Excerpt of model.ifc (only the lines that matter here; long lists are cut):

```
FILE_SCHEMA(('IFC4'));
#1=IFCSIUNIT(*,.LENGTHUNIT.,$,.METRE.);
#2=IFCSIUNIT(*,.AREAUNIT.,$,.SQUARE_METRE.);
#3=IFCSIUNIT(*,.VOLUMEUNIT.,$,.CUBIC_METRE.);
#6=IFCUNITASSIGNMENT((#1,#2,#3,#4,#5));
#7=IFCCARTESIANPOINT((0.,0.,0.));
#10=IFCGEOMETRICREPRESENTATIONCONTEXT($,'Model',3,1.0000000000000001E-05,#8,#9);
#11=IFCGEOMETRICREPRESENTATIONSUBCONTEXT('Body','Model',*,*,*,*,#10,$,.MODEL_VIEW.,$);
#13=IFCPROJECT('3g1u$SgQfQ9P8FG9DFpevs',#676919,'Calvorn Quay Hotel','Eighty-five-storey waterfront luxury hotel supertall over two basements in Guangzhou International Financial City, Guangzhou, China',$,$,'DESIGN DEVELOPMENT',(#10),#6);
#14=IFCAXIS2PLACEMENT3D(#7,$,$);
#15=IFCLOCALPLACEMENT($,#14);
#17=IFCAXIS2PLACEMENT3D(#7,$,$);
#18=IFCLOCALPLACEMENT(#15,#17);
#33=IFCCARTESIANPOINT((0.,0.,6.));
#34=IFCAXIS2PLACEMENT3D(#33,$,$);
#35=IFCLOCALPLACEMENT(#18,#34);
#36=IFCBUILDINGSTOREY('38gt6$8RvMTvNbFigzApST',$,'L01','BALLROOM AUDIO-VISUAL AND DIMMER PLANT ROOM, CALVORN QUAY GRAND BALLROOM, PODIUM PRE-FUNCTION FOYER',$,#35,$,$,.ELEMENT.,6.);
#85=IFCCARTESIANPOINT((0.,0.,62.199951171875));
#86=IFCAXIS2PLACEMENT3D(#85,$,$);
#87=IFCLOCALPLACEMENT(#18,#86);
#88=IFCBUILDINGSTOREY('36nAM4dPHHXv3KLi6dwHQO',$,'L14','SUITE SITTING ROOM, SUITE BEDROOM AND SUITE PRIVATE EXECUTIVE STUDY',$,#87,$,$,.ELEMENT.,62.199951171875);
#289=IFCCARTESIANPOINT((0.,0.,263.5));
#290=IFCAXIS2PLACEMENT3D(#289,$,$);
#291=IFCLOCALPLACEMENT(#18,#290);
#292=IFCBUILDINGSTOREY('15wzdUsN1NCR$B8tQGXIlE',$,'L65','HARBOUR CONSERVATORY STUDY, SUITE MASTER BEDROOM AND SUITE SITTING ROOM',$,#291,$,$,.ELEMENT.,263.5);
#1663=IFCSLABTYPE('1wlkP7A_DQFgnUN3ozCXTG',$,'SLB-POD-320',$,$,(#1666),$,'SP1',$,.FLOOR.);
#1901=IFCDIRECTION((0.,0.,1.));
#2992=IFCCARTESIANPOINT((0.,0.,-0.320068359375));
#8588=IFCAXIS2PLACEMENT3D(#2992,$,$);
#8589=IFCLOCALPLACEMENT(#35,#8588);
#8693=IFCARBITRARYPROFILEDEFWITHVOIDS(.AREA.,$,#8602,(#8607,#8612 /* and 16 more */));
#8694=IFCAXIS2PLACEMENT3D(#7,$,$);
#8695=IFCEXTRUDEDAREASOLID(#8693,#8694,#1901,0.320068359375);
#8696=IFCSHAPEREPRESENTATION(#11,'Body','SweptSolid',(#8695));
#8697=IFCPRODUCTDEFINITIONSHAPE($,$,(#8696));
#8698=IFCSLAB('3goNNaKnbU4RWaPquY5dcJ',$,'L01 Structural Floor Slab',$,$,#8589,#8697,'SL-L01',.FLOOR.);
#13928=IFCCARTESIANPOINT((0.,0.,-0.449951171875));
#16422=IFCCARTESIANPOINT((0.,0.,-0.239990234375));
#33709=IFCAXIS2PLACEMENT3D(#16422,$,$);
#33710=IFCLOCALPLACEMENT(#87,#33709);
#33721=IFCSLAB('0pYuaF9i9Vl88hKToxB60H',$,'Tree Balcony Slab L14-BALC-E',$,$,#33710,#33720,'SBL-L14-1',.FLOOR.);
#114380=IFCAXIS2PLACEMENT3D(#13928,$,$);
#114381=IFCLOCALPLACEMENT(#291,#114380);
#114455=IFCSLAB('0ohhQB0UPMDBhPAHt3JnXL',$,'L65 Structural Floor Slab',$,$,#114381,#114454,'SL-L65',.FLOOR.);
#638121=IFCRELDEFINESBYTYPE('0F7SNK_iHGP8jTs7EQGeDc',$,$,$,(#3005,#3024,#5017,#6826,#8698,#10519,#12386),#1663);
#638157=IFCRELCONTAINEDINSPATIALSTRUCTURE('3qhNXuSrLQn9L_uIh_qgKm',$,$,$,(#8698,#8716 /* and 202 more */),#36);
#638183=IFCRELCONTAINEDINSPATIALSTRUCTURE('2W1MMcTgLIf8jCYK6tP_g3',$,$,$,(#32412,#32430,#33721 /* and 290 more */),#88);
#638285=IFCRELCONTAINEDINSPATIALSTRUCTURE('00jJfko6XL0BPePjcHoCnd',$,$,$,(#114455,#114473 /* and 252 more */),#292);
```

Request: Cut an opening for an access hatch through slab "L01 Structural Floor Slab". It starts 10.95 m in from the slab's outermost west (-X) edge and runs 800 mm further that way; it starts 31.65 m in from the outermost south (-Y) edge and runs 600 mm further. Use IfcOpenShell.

```python
import numpy as np
import ifcopenshell
import ifcopenshell.api.feature
import ifcopenshell.api.geometry
import ifcopenshell.api.root
import ifcopenshell.geom
import ifcopenshell.util.placement
import ifcopenshell.util.representation
import ifcopenshell.util.shape
import ifcopenshell.util.unit

model = ifcopenshell.open("model.ifc")
unit_scale = ifcopenshell.util.unit.calculate_unit_scale(model)
settings = ifcopenshell.geom.settings()


def volume(element):
    """Net volume in cubic metres, openings subtracted."""
    shape = ifcopenshell.geom.create_shape(settings, element)
    return ifcopenshell.util.shape.get_volume(shape.geometry)


slab = model.by_guid("3goNNaKnbU4RWaPquY5dcJ")
before = volume(slab)

# Extent in the slab's own axes, in metres. The edges named are its -X and -Y sides.
slab_shape = ifcopenshell.geom.create_shape(settings, slab)
vertices = ifcopenshell.util.shape.get_vertices(slab_shape.geometry)
x_min, y_min, bottom = vertices.min(axis=0)
top = vertices[:, 2].max()

opening = ifcopenshell.api.root.create_entity(model, ifc_class="IfcOpeningElement", name="Access hatch opening", predefined_type="OPENING")
context = ifcopenshell.util.representation.get_context(model, "Model", "Body", "MODEL_VIEW")
width, depth = 0.8, 0.6
outline = [(0.0, 0.0), (width, 0.0), (width, depth), (0.0, depth), (0.0, 0.0)]
# Overshoot both faces by 50 mm so the cut is clean.
shape = ifcopenshell.api.geometry.add_slab_representation(
    model, context=context, depth=top - bottom + 0.1, polyline=outline
)
ifcopenshell.api.geometry.assign_representation(model, product=opening, representation=shape)

matrix = ifcopenshell.util.placement.get_local_placement(slab.ObjectPlacement)
matrix[:, 3] = matrix @ np.append(np.array([x_min + 10.95, y_min + 31.65, bottom - 0.05]) / unit_scale, 1.0)
ifcopenshell.api.geometry.edit_object_placement(model, product=opening, matrix=matrix, is_si=False)
ifcopenshell.api.feature.add_feature(model, feature=opening, element=slab)

after = volume(slab)

print(f"slab volume {before:.3f} -> {after:.3f} m3")

model.write("model-out.ifc")
```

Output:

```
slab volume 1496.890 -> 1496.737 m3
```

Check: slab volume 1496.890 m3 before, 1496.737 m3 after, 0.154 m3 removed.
